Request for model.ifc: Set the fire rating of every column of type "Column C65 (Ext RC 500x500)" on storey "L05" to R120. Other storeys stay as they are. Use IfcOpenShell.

First a look at what the model holds.

```python
import ifcopenshell
import ifcopenshell.util.element

model = ifcopenshell.open("model.ifc")
print(model.schema)
storey = next(s for s in model.by_type("IfcBuildingStorey") if s.Name == "L05")
columns = [e for e in ifcopenshell.util.element.get_decomposition(storey) if e.is_a("IfcColumn")]
seen = {}
for e in columns:
    element_type = ifcopenshell.util.element.get_type(e)
    key = (element_type.Name if element_type != e and element_type else None, ifcopenshell.util.element.get_pset(e, "Pset_ColumnCommon", "FireRating"))
    seen[key] = seen.get(key, 0) + 1
for (name, value), count in sorted(seen.items(), key=str):
    print(count, "x", name, "|", value)
```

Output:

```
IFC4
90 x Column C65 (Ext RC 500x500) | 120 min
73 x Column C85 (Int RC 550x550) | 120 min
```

```python
import ifcopenshell
import ifcopenshell.api.pset
import ifcopenshell.util.element

model = ifcopenshell.open("model.ifc")

storey = next(s for s in model.by_type("IfcBuildingStorey") if s.Name == "L05")
columns = [e for e in ifcopenshell.util.element.get_decomposition(storey) if e.is_a("IfcColumn")]

count = 0
for e in columns:
    element_type = ifcopenshell.util.element.get_type(e)
    if element_type in (None, e) or element_type.Name != "Column C65 (Ext RC 500x500)":
        continue
    # add_pset returns the element's existing set when there is one.
    pset = ifcopenshell.api.pset.add_pset(model, product=e, name="Pset_ColumnCommon")
    ifcopenshell.api.pset.edit_pset(model, pset=pset, properties={"FireRating": "R120"})
    count += 1

print(count, "columns updated")

model.write("model-out.ifc")
```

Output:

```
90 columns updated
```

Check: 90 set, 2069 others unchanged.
